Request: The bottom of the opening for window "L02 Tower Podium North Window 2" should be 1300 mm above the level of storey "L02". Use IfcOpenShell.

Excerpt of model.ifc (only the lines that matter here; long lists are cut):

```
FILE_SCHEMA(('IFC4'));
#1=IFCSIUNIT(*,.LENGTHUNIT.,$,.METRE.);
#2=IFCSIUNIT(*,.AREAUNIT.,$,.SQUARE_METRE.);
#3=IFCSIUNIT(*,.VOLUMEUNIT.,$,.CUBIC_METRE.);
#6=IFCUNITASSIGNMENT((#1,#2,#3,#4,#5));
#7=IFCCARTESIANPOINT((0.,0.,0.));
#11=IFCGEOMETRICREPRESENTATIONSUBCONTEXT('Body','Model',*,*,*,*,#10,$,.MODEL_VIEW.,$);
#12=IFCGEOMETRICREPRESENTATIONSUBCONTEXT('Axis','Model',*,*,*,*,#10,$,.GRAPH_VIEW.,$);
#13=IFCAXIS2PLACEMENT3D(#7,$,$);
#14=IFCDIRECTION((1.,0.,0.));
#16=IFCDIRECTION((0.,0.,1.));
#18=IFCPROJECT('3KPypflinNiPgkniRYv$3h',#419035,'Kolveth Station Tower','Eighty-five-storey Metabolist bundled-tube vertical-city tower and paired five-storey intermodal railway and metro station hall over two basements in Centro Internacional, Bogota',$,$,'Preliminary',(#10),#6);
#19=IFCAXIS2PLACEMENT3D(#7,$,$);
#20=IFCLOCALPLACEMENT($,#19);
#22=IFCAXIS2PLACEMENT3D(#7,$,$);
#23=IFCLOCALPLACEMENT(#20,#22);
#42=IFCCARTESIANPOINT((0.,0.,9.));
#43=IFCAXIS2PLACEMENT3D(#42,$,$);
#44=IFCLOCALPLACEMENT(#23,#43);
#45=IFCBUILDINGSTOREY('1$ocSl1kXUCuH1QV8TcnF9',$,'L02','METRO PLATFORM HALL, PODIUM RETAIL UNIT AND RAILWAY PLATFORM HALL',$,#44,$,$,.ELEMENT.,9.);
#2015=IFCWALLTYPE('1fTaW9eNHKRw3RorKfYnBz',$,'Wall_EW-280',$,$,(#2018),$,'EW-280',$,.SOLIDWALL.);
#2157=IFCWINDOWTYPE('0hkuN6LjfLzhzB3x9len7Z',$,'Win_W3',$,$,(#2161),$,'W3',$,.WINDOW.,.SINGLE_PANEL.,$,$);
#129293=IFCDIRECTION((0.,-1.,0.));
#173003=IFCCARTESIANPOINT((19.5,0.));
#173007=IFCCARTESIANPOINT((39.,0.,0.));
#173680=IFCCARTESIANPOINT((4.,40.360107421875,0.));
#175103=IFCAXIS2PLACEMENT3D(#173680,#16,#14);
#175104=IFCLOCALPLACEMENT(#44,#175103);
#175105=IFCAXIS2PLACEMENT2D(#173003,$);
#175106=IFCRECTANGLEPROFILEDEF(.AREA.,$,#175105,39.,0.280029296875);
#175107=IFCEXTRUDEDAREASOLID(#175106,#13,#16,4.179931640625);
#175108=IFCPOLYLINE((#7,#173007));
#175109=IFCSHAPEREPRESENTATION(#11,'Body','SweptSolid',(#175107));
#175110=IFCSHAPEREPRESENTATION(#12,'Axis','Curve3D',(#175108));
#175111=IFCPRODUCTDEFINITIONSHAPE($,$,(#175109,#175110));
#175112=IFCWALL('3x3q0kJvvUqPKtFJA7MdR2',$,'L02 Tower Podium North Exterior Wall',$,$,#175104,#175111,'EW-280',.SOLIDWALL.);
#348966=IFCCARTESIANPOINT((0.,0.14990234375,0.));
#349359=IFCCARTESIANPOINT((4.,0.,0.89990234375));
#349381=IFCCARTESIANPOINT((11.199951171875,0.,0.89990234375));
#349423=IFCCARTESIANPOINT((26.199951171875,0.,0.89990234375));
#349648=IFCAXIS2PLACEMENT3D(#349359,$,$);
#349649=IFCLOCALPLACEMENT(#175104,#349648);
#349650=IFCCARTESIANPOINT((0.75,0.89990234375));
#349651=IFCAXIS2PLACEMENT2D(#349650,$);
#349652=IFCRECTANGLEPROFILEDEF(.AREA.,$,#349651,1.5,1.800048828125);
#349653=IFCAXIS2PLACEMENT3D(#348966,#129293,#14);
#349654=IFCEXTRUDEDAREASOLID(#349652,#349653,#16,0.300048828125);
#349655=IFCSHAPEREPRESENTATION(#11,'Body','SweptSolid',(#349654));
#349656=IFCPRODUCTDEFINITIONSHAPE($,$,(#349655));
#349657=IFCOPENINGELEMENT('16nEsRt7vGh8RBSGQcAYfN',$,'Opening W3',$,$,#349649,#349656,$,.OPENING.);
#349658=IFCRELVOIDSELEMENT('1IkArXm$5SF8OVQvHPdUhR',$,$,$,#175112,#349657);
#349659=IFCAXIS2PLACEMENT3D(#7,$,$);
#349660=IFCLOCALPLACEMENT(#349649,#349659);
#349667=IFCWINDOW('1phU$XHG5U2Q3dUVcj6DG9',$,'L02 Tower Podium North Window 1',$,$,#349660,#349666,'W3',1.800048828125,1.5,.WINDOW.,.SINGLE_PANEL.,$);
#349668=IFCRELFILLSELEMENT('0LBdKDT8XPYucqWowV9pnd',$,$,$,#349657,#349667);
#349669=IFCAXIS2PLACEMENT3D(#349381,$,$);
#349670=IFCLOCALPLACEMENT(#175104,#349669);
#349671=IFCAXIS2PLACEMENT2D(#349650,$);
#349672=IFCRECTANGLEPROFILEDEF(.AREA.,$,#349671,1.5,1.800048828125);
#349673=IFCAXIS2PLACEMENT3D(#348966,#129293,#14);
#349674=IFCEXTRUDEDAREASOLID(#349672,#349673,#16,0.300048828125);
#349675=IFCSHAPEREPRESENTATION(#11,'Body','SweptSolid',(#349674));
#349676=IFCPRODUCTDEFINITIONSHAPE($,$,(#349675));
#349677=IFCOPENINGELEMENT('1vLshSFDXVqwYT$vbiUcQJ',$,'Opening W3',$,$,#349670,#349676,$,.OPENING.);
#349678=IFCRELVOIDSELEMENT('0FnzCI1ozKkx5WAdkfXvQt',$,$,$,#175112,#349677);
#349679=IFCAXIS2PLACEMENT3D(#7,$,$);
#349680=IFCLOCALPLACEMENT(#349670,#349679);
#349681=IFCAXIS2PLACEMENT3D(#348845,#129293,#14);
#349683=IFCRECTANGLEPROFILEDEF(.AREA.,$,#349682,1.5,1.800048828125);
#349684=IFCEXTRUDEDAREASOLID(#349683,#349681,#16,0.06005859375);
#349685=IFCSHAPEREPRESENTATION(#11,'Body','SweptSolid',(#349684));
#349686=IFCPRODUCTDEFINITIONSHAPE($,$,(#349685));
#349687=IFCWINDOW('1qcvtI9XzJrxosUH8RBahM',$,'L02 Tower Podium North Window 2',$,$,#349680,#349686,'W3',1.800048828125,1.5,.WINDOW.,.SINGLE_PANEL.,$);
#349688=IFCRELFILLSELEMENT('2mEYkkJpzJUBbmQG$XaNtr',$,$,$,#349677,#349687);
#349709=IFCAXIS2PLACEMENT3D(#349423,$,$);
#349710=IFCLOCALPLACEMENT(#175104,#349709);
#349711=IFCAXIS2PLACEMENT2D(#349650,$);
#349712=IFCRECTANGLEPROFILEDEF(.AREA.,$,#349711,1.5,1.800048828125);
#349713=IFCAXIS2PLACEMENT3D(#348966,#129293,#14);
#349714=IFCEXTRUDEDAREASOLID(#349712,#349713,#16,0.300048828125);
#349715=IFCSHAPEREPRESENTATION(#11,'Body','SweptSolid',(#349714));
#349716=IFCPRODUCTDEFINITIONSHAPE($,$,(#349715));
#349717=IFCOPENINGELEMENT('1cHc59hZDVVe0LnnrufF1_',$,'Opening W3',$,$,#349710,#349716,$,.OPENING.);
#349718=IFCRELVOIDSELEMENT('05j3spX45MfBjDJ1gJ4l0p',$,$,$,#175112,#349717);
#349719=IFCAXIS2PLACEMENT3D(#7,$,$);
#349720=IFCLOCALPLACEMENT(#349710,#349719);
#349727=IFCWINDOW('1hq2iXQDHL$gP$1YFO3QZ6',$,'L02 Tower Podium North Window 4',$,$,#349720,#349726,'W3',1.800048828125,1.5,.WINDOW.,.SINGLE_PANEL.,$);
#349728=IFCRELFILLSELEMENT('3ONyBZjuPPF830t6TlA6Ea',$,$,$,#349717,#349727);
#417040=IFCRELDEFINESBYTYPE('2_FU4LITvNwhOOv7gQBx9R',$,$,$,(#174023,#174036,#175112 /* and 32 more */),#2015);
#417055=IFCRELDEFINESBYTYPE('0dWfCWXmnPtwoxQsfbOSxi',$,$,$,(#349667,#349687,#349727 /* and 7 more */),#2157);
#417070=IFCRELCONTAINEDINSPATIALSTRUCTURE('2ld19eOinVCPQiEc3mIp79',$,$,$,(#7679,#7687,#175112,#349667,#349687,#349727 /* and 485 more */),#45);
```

```python
import numpy as np
import ifcopenshell
import ifcopenshell.api.geometry
import ifcopenshell.geom
import ifcopenshell.util.element
import ifcopenshell.util.placement
import ifcopenshell.util.shape
import ifcopenshell.util.unit

model = ifcopenshell.open("model.ifc")
unit_scale = ifcopenshell.util.unit.calculate_unit_scale(model)

window = model.by_guid("1qcvtI9XzJrxosUH8RBahM")
opening = window.FillsVoids[0].RelatingOpeningElement
storey = ifcopenshell.util.element.get_container(window, ifc_class="IfcBuildingStorey")
level = ifcopenshell.util.placement.get_local_placement(storey.ObjectPlacement)[2, 3]

# The opening's origin need not be at the sill, so measure its lowest point.
shape = ifcopenshell.geom.create_shape(ifcopenshell.geom.settings(), opening)
bottom = ifcopenshell.util.shape.get_shape_bottom_elevation(shape, shape.geometry) / unit_scale
dz = level + 1.3 / unit_scale - bottom

shift = np.array([0.0, 0.0, dz])
# The window is placed relative to its opening, so it follows when the opening moves.
matrix = ifcopenshell.util.placement.get_local_placement(opening.ObjectPlacement)
matrix[:3, 3] += shift
ifcopenshell.api.geometry.edit_object_placement(
    model, product=opening, matrix=matrix, is_si=False, should_transform_children=True
)

print(f"moved by {dz * unit_scale:+.3f} m")

model.write("model-out.ifc")
```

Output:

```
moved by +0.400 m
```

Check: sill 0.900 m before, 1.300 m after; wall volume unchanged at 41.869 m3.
